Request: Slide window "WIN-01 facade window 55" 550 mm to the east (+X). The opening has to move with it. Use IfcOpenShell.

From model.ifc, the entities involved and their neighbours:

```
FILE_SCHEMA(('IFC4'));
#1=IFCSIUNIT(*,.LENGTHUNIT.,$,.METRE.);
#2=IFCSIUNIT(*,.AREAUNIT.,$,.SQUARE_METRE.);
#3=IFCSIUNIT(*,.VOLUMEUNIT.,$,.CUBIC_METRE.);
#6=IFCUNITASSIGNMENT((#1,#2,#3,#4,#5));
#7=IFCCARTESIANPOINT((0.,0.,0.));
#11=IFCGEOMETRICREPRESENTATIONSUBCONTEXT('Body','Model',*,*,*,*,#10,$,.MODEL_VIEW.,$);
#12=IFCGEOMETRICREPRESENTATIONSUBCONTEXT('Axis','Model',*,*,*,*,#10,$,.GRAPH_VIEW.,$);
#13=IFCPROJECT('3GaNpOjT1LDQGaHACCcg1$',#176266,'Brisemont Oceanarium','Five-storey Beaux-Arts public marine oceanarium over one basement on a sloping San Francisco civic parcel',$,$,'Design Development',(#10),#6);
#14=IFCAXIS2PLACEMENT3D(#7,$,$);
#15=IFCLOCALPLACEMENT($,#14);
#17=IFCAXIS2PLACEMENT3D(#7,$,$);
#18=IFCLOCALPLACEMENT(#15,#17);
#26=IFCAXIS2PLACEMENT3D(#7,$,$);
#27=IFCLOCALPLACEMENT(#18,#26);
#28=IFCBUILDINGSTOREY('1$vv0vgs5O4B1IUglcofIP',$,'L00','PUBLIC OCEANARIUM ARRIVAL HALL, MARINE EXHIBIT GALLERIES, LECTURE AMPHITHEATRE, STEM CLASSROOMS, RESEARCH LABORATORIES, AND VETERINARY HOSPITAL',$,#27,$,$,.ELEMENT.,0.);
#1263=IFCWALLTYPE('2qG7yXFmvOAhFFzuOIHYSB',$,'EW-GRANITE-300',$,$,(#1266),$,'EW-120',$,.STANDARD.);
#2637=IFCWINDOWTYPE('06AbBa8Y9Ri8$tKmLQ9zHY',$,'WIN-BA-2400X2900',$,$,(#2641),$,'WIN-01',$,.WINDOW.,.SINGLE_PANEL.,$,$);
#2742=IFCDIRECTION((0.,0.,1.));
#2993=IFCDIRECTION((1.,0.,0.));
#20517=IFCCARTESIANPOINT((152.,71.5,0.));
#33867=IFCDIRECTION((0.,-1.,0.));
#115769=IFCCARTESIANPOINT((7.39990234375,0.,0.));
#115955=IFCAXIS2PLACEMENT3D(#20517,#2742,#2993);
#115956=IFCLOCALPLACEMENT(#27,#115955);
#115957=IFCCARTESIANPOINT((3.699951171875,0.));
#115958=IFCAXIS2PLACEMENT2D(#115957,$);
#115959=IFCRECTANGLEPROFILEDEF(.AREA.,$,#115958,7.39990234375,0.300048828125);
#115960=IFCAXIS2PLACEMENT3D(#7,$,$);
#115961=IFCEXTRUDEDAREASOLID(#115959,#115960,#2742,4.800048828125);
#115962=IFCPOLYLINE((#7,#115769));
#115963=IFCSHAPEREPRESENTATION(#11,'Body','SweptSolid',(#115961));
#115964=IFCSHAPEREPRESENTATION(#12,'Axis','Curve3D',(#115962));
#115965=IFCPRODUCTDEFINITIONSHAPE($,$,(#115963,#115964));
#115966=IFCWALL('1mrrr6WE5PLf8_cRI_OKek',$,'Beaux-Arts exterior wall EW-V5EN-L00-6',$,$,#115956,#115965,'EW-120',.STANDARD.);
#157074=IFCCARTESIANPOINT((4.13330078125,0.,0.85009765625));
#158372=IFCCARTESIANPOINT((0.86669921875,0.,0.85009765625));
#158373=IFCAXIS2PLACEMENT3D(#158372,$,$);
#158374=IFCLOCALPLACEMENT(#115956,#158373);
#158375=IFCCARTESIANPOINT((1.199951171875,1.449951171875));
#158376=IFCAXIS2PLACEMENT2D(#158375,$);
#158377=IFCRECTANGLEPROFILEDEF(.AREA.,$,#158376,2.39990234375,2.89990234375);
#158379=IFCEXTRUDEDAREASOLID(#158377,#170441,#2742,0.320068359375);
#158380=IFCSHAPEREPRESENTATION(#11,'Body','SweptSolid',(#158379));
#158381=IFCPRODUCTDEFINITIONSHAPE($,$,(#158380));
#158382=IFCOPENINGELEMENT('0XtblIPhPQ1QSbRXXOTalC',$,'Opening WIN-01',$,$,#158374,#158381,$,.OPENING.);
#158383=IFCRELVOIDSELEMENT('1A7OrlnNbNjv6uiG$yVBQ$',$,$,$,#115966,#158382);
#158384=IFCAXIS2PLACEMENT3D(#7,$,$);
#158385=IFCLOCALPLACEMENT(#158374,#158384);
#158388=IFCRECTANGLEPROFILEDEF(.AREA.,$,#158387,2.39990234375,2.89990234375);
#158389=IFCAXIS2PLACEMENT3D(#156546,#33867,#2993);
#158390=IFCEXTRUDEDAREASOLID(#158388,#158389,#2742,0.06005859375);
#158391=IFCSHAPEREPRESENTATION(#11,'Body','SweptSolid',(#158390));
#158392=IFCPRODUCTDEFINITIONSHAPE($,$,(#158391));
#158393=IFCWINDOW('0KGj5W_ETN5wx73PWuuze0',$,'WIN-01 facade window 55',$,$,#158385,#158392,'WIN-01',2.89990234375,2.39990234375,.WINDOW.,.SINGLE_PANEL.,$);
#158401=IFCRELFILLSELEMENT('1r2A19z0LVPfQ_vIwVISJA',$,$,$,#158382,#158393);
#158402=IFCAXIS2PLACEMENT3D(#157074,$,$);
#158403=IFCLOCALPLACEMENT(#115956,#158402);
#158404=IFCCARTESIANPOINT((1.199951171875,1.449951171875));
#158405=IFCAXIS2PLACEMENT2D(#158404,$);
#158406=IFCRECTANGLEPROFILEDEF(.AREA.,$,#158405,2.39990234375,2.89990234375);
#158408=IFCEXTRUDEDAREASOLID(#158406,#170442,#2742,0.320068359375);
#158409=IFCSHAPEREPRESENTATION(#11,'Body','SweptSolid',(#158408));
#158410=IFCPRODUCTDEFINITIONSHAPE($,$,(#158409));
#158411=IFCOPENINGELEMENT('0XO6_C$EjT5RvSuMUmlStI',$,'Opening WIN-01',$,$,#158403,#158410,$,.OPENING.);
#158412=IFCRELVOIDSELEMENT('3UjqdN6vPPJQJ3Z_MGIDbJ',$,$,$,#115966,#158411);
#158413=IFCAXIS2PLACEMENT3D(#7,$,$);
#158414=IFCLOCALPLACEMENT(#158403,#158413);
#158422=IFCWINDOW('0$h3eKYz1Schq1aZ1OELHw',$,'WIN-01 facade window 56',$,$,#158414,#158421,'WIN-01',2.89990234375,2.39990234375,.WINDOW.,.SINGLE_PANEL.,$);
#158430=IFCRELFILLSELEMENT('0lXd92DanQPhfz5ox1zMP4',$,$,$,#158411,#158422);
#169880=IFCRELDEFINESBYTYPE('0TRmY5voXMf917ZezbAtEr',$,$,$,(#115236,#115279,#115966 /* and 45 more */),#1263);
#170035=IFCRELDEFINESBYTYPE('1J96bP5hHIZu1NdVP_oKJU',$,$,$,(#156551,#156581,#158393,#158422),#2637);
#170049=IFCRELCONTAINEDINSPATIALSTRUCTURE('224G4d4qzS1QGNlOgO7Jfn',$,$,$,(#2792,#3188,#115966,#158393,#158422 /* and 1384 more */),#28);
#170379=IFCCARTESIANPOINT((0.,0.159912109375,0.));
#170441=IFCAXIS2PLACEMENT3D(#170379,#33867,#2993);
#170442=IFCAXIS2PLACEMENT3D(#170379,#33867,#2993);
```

```python
import ifcopenshell
import ifcopenshell.api.geometry
import ifcopenshell.util.placement

model = ifcopenshell.open("model.ifc")

window = model.by_guid("0KGj5W_ETN5wx73PWuuze0")
opening = window.FillsVoids[0].RelatingOpeningElement
wall = opening.VoidsElements[0].RelatingBuildingElement

wall_matrix = ifcopenshell.util.placement.get_local_placement(wall.ObjectPlacement)
shift = wall_matrix[:3, 0] * 0.55
before = ifcopenshell.util.placement.get_local_placement(window.ObjectPlacement)[:3, 3].copy()

# The window is placed relative to its opening, so it follows when the opening moves.
matrix = ifcopenshell.util.placement.get_local_placement(opening.ObjectPlacement)
matrix[:3, 3] += shift
ifcopenshell.api.geometry.edit_object_placement(
    model, product=opening, matrix=matrix, is_si=False, should_transform_children=True
)

after = ifcopenshell.util.placement.get_local_placement(window.ObjectPlacement)[:3, 3]
print("window moved by", (after - before).round(3) + 0.0)

model.write("model_rev.ifc")
```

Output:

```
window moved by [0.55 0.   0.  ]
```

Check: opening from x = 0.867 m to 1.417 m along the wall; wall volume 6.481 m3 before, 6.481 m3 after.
